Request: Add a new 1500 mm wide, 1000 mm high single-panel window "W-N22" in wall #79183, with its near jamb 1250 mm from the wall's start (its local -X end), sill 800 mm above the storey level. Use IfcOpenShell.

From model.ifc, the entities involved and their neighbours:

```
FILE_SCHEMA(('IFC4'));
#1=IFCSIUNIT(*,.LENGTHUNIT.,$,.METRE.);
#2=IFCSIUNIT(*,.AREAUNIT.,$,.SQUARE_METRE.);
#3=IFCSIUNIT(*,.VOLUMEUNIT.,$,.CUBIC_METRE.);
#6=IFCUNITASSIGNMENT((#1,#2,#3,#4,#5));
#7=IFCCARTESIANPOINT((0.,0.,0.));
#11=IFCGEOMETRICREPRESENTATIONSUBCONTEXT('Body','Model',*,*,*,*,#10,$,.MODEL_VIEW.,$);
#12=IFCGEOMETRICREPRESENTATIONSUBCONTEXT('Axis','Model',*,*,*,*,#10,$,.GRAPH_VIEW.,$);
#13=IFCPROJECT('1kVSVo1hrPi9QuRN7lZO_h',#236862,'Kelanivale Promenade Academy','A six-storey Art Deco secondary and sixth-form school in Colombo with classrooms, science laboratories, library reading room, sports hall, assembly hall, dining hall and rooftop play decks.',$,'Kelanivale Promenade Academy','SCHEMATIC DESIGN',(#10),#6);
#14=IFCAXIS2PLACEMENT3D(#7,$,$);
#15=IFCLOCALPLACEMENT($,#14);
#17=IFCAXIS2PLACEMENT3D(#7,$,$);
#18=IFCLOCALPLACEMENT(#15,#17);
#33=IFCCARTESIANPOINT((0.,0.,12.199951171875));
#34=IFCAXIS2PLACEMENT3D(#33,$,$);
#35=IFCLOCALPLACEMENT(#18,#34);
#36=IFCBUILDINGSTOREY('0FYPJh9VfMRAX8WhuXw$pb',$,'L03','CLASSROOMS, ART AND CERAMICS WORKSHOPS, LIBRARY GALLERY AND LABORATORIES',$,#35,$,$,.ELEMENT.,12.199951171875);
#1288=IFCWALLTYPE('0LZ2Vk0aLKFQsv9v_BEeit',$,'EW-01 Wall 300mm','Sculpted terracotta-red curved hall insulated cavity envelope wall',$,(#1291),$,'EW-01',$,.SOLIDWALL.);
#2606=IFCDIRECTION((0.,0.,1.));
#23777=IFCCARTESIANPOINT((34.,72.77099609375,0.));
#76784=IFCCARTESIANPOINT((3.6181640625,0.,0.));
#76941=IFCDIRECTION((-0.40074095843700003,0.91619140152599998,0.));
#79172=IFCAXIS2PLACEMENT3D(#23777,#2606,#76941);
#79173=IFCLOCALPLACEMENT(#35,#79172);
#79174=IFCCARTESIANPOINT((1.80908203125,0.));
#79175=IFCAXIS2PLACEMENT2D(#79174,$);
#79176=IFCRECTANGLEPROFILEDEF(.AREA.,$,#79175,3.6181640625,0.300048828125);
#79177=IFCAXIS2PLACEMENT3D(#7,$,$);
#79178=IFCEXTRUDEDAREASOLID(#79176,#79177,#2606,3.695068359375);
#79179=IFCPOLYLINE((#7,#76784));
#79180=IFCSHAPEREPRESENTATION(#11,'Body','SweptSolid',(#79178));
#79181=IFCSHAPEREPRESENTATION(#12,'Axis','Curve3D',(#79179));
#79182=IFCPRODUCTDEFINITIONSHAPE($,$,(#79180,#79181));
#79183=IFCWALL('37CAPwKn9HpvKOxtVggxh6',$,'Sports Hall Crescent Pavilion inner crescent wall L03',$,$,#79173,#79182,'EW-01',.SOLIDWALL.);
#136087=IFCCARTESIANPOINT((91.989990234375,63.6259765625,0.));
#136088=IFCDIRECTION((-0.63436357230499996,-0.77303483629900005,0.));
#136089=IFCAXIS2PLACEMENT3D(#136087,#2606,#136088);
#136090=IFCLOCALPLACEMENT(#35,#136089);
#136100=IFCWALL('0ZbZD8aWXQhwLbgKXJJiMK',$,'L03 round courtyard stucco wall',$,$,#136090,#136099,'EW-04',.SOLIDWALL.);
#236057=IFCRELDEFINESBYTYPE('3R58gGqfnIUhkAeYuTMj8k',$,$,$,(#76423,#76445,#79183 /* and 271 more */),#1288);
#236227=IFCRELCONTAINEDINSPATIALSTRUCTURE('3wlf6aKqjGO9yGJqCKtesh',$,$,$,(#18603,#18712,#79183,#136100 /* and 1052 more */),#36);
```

```python
import numpy as np
import ifcopenshell
import ifcopenshell.api.feature
import ifcopenshell.api.geometry
import ifcopenshell.api.root
import ifcopenshell.api.spatial
import ifcopenshell.geom
import ifcopenshell.util.element
import ifcopenshell.util.placement
import ifcopenshell.util.representation
import ifcopenshell.util.shape
import ifcopenshell.util.unit

model = ifcopenshell.open("model.ifc")
unit_scale = ifcopenshell.util.unit.calculate_unit_scale(model)
settings = ifcopenshell.geom.settings()


def volume(element):
    """Net volume in cubic metres, openings subtracted."""
    shape = ifcopenshell.geom.create_shape(settings, element)
    return ifcopenshell.util.shape.get_volume(shape.geometry)


wall = model.by_id(79183)
storey = ifcopenshell.util.element.get_container(wall, ifc_class="IfcBuildingStorey")
context = ifcopenshell.util.representation.get_context(model, "Model", "Body", "MODEL_VIEW")
before = volume(wall)

width, height, from_end, sill = 1.5, 1, 1.25, 0.8  # metres

# The wall runs along its own X axis, and the end named is its -X end.
wall_shape = ifcopenshell.geom.create_shape(settings, wall)
x, y, z = ifcopenshell.util.shape.get_vertices(wall_shape.geometry).T
start = x.min() + from_end
face, thickness = float(y.min()), float(y.max() - y.min())
wall_matrix = ifcopenshell.util.placement.get_local_placement(wall.ObjectPlacement)
level = ifcopenshell.util.placement.get_local_placement(storey.ObjectPlacement)[2, 3]


def in_wall(x, y):
    """Placement at x, y metres in the wall's axes, at sill height."""
    matrix = wall_matrix.copy()
    matrix[:, 3] = wall_matrix @ np.array([x / unit_scale, y / unit_scale, 0.0, 1.0])
    matrix[2, 3] = level + sill / unit_scale
    return matrix


# Opening: a box that overshoots both wall faces by 50 mm.
opening = ifcopenshell.api.root.create_entity(model, ifc_class="IfcOpeningElement", predefined_type="OPENING")
box = ifcopenshell.api.geometry.add_wall_representation(
    model, context=context, length=width, height=height, thickness=thickness + 0.1
)
ifcopenshell.api.geometry.assign_representation(model, product=opening, representation=box)
ifcopenshell.api.geometry.edit_object_placement(model, product=opening, matrix=in_wall(start, face - 0.05), is_si=False)
ifcopenshell.api.feature.add_feature(model, feature=opening, element=wall)

window = ifcopenshell.api.root.create_entity(model, ifc_class="IfcWindow", name="W-N22", predefined_type="WINDOW")
window.OverallWidth, window.OverallHeight = width / unit_scale, height / unit_scale
window.PartitioningType = "SINGLE_PANEL"
body = ifcopenshell.api.geometry.add_window_representation(
    model,
    context=context,
    overall_width=window.OverallWidth,
    overall_height=window.OverallHeight,
    partition_type="SINGLE_PANEL",
)
ifcopenshell.api.geometry.assign_representation(model, product=window, representation=body)
ifcopenshell.api.spatial.assign_container(model, products=[window], relating_structure=storey)
ifcopenshell.api.feature.add_filling(model, opening=opening, element=window)

# Centre the window in the wall's thickness.
ifcopenshell.api.geometry.edit_object_placement(model, product=window, matrix=in_wall(start, face), is_si=False)
window_shape = ifcopenshell.geom.create_shape(settings, window)
depth = ifcopenshell.util.shape.get_vertices(window_shape.geometry)[:, 1]
offset = face + thickness / 2 - (depth.min() + depth.max()) / 2
ifcopenshell.api.geometry.edit_object_placement(model, product=window, matrix=in_wall(start, offset), is_si=False)

after = volume(wall)

print(f"wall volume {before:.3f} -> {after:.3f} m3")

model.write("model_edited.ifc")
```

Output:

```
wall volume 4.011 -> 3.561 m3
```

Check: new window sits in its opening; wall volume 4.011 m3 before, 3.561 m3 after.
